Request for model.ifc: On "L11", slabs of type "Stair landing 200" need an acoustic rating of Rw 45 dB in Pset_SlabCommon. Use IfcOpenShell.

First a look at what the model holds.

```python
import ifcopenshell
import ifcopenshell.util.element

model = ifcopenshell.open("model.ifc")
print(model.schema)
storey = next(s for s in model.by_type("IfcBuildingStorey") if s.Name == "L11")
slabs = [e for e in ifcopenshell.util.element.get_decomposition(storey) if e.is_a("IfcSlab")]
seen = {}
for e in slabs:
    element_type = ifcopenshell.util.element.get_type(e)
    key = (element_type.Name if element_type != e and element_type else None, ifcopenshell.util.element.get_pset(e, "Pset_SlabCommon", "AcousticRating"))
    seen[key] = seen.get(key, 0) + 1
for (name, value), count in sorted(seen.items(), key=str):
    print(count, "x", name, "|", value)
```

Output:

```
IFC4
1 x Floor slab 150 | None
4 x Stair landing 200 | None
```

```python
import ifcopenshell
import ifcopenshell.api.pset
import ifcopenshell.util.element

model = ifcopenshell.open("model.ifc")

storey = next(s for s in model.by_type("IfcBuildingStorey") if s.Name == "L11")
slabs = [e for e in ifcopenshell.util.element.get_decomposition(storey) if e.is_a("IfcSlab")]

count = 0
for e in slabs:
    element_type = ifcopenshell.util.element.get_type(e)
    if element_type in (None, e) or element_type.Name != "Stair landing 200":
        continue
    found = ifcopenshell.util.element.get_pset(e, "Pset_SlabCommon", should_inherit=False)
    if found:
        pset = model.by_id(found["id"])
        if len(ifcopenshell.util.element.get_elements_by_pset(pset)) > 1:
            pset = ifcopenshell.api.pset.unshare_pset(model, products=[e], pset=pset)[0]
    else:
        pset = ifcopenshell.api.pset.add_pset(model, product=e, name="Pset_SlabCommon")
    ifcopenshell.api.pset.edit_pset(model, pset=pset, properties={"AcousticRating": "Rw 45 dB"})
    count += 1

print(count, "slabs updated")

model.write("model_updated.ifc")
```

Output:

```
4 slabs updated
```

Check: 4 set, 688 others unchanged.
